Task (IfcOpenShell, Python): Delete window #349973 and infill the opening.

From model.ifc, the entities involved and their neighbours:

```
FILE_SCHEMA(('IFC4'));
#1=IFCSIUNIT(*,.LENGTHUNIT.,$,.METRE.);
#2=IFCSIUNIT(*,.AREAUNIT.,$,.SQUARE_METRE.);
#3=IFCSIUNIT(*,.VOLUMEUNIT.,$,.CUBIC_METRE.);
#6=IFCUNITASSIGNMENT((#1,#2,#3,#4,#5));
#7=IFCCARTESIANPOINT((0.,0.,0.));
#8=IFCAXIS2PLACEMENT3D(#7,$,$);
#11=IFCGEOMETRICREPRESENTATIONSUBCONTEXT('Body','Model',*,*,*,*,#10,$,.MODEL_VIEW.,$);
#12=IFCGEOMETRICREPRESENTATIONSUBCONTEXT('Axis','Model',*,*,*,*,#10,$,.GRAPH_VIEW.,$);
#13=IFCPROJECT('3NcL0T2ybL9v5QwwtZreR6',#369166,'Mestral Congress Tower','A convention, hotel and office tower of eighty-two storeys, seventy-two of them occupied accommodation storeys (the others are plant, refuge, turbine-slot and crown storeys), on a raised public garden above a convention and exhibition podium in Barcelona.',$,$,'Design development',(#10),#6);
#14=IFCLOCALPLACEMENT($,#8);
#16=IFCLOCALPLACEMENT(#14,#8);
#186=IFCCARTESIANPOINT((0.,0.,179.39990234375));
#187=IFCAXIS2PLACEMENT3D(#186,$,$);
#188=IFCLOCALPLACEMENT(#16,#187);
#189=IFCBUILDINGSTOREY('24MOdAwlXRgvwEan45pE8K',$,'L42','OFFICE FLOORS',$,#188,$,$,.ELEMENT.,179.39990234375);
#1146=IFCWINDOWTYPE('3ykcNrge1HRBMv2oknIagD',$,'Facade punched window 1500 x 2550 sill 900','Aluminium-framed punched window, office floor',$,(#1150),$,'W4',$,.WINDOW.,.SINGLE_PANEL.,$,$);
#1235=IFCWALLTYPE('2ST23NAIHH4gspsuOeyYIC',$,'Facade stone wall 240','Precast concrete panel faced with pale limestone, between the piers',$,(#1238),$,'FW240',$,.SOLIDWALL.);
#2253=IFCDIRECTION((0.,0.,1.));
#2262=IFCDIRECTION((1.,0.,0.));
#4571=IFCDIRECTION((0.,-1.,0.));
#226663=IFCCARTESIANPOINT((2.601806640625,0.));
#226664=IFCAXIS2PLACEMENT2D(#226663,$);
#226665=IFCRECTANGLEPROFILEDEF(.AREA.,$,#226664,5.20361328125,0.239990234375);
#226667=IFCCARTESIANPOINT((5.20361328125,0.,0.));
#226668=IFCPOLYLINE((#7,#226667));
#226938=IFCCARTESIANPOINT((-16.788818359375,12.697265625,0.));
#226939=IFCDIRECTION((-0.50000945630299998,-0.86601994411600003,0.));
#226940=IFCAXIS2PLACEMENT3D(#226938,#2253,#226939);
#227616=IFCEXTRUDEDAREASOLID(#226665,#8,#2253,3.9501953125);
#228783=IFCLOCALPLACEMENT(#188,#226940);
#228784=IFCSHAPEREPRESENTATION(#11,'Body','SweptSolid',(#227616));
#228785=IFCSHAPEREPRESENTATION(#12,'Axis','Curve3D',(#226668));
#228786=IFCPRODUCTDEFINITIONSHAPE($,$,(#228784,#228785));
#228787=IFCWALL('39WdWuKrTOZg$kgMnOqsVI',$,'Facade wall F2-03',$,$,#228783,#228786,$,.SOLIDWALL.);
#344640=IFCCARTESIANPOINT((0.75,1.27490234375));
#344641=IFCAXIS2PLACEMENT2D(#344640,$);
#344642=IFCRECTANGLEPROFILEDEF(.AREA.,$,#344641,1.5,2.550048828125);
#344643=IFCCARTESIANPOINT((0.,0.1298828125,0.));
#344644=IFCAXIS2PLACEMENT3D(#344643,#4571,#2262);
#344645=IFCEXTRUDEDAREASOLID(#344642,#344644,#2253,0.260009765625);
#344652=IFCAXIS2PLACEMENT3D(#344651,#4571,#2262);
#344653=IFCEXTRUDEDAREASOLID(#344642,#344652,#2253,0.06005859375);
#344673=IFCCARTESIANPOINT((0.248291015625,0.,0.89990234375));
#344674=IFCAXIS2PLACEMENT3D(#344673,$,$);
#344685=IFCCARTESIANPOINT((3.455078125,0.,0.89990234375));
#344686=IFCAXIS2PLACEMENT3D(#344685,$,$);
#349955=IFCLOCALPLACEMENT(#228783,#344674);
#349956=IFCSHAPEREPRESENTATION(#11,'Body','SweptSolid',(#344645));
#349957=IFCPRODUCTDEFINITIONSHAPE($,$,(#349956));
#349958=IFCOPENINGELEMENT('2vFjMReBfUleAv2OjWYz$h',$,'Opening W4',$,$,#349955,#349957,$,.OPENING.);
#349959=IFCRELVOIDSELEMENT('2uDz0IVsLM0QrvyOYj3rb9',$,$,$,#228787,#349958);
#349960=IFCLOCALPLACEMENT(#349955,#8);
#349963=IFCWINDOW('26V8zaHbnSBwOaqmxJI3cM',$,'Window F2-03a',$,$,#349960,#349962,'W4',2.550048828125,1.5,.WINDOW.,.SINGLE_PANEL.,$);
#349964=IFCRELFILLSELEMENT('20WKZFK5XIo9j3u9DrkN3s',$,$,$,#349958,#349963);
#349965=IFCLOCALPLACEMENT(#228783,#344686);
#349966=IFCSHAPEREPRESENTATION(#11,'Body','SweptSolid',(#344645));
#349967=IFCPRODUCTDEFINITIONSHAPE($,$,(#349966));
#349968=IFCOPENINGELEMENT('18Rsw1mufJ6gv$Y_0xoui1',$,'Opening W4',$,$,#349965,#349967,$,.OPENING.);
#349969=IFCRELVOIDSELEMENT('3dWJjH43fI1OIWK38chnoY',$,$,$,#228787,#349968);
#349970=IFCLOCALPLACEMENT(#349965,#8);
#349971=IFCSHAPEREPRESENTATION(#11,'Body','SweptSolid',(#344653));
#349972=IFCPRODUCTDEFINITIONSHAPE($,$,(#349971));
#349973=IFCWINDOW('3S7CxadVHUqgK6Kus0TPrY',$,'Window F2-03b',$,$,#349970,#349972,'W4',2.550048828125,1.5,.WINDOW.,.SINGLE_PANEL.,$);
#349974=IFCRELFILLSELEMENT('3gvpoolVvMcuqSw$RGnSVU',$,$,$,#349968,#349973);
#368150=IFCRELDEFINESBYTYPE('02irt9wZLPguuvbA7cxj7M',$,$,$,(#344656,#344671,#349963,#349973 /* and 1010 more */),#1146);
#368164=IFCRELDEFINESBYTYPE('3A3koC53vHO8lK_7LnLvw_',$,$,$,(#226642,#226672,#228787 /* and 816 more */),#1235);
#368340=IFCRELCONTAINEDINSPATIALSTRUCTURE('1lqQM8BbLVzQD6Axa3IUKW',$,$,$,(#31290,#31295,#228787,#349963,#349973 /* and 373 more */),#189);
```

```python
import ifcopenshell
import ifcopenshell.api.feature
import ifcopenshell.api.root
import ifcopenshell.geom
import ifcopenshell.util.shape

model = ifcopenshell.open("model.ifc")
settings = ifcopenshell.geom.settings()


def volume(element):
    """Net volume in cubic metres, openings subtracted."""
    shape = ifcopenshell.geom.create_shape(settings, element)
    return ifcopenshell.util.shape.get_volume(shape.geometry)


window = model.by_id(349973)
opening = window.FillsVoids[0].RelatingOpeningElement
wall = opening.VoidsElements[0].RelatingBuildingElement
before = volume(wall)

ifcopenshell.api.root.remove_product(model, product=window)
ifcopenshell.api.feature.remove_feature(model, feature=opening)

after = volume(wall)

print(f"wall volume {before:.3f} -> {after:.3f} m3")

model.write("model_updated.ifc")
```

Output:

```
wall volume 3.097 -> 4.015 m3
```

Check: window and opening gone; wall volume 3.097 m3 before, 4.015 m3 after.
